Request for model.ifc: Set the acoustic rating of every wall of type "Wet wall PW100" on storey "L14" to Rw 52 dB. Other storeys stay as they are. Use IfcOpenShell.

First a look at what the model holds.

```python
import ifcopenshell
import ifcopenshell.util.element

model = ifcopenshell.open("model.ifc")
print(model.schema)
storey = next(s for s in model.by_type("IfcBuildingStorey") if s.Name == "L14")
walls = [e for e in ifcopenshell.util.element.get_decomposition(storey) if e.is_a("IfcWall")]
seen = {}
for e in walls:
    element_type = ifcopenshell.util.element.get_type(e)
    key = (element_type.Name if element_type != e and element_type else None, ifcopenshell.util.element.get_pset(e, "Pset_WallCommon", "AcousticRating"))
    seen[key] = seen.get(key, 0) + 1
for (name, value), count in sorted(seen.items(), key=str):
    print(count, "x", name, "|", value)
```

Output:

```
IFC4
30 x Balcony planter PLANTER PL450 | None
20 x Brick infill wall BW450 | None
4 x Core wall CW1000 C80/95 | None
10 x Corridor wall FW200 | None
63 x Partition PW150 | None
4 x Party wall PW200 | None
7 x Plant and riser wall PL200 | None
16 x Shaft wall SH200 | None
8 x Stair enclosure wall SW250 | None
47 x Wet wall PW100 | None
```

```python
import ifcopenshell
import ifcopenshell.api.pset
import ifcopenshell.util.element

model = ifcopenshell.open("model.ifc")

storey = next(s for s in model.by_type("IfcBuildingStorey") if s.Name == "L14")
walls = [e for e in ifcopenshell.util.element.get_decomposition(storey) if e.is_a("IfcWall")]

count = 0
for e in walls:
    element_type = ifcopenshell.util.element.get_type(e)
    if element_type in (None, e) or element_type.Name != "Wet wall PW100":
        continue
    found = ifcopenshell.util.element.get_pset(e, "Pset_WallCommon", should_inherit=False)
    if found:
        pset = model.by_id(found["id"])
        if len(ifcopenshell.util.element.get_elements_by_pset(pset)) > 1:
            pset = ifcopenshell.api.pset.unshare_pset(model, products=[e], pset=pset)[0]
    else:
        pset = ifcopenshell.api.pset.add_pset(model, product=e, name="Pset_WallCommon")
    ifcopenshell.api.pset.edit_pset(model, pset=pset, properties={"AcousticRating": "Rw 52 dB"})
    count += 1

print(count, "walls updated")

model.write("model_v2.ifc")
```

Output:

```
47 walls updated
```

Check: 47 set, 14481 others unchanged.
